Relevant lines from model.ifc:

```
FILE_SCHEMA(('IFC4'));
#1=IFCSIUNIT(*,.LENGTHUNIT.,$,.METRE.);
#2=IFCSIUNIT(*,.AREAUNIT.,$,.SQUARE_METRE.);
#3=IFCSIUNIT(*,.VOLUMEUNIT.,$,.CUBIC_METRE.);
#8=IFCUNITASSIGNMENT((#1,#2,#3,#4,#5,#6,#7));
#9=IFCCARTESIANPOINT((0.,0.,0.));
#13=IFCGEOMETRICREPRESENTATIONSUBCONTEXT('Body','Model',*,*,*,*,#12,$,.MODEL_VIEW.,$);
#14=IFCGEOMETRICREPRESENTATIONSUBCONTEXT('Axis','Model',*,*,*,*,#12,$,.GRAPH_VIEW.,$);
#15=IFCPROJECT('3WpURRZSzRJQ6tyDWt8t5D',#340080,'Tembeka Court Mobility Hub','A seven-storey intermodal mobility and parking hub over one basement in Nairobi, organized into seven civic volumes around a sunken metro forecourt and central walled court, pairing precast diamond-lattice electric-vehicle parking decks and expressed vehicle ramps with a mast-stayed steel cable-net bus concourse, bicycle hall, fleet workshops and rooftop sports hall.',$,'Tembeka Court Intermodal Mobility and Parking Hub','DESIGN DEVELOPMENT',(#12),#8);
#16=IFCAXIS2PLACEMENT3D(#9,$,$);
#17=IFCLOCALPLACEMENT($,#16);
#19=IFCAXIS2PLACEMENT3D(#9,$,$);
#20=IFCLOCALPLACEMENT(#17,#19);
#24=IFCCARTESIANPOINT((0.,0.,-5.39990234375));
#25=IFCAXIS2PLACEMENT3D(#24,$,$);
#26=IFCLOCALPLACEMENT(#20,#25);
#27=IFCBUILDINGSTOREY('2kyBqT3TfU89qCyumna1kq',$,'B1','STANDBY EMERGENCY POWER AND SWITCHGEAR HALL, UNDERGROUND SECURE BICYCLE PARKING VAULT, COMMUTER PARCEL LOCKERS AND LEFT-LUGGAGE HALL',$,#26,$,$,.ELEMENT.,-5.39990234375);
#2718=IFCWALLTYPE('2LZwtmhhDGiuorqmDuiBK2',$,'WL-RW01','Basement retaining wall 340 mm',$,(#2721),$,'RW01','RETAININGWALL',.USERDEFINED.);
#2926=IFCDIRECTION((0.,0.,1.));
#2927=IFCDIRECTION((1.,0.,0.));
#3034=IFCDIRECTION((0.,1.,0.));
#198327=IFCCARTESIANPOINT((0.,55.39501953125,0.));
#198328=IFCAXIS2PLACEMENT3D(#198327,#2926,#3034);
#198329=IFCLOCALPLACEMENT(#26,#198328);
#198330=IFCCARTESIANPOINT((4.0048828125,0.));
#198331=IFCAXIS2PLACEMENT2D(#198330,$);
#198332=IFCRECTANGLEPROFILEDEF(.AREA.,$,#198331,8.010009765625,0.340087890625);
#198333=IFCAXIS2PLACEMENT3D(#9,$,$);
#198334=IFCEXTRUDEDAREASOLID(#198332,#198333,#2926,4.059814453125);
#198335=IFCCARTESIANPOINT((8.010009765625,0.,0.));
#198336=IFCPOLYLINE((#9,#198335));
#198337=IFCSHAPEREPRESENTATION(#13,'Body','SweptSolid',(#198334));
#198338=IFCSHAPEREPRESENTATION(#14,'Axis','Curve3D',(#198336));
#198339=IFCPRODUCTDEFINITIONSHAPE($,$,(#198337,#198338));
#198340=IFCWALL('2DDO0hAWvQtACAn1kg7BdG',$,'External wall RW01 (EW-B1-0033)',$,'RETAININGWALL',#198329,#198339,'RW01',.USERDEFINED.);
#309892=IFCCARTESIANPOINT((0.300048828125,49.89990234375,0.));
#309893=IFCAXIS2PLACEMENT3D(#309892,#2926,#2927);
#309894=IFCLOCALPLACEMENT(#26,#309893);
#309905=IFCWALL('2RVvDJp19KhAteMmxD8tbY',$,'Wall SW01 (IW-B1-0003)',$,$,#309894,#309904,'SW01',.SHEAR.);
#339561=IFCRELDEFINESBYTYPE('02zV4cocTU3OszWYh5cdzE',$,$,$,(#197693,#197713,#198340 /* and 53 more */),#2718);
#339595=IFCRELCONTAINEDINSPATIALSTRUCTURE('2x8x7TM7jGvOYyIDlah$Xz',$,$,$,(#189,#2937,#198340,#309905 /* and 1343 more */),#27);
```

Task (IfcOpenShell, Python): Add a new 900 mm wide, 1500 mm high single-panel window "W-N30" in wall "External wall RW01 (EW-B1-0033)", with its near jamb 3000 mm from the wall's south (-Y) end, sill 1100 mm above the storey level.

```python
import numpy as np
import ifcopenshell
import ifcopenshell.api.feature
import ifcopenshell.api.geometry
import ifcopenshell.api.root
import ifcopenshell.api.spatial
import ifcopenshell.geom
import ifcopenshell.util.element
import ifcopenshell.util.placement
import ifcopenshell.util.representation
import ifcopenshell.util.shape
import ifcopenshell.util.unit

model = ifcopenshell.open("model.ifc")
unit_scale = ifcopenshell.util.unit.calculate_unit_scale(model)
settings = ifcopenshell.geom.settings()


def volume(element):
    """Net volume in cubic metres, openings subtracted."""
    shape = ifcopenshell.geom.create_shape(settings, element)
    return ifcopenshell.util.shape.get_volume(shape.geometry)


wall = model.by_id(198340)
storey = ifcopenshell.util.element.get_container(wall, ifc_class="IfcBuildingStorey")
context = ifcopenshell.util.representation.get_context(model, "Model", "Body", "MODEL_VIEW")
before = volume(wall)

width, height, from_end, sill = 0.9, 1.5, 3, 1.1  # metres

# The wall runs along its own X axis, and the end named is its -X end.
wall_shape = ifcopenshell.geom.create_shape(settings, wall)
x, y, z = ifcopenshell.util.shape.get_vertices(wall_shape.geometry).T
start = x.min() + from_end
face, thickness = float(y.min()), float(y.max() - y.min())
wall_matrix = ifcopenshell.util.placement.get_local_placement(wall.ObjectPlacement)
level = ifcopenshell.util.placement.get_local_placement(storey.ObjectPlacement)[2, 3]


def in_wall(x, y):
    """Placement at x, y metres in the wall's axes, at sill height."""
    matrix = wall_matrix.copy()
    matrix[:, 3] = wall_matrix @ np.array([x / unit_scale, y / unit_scale, 0.0, 1.0])
    matrix[2, 3] = level + sill / unit_scale
    return matrix


# Opening: a box that overshoots both wall faces by 50 mm.
opening = ifcopenshell.api.root.create_entity(model, ifc_class="IfcOpeningElement", predefined_type="OPENING")
box = ifcopenshell.api.geometry.add_wall_representation(
    model, context=context, length=width, height=height, thickness=thickness + 0.1
)
ifcopenshell.api.geometry.assign_representation(model, product=opening, representation=box)
ifcopenshell.api.geometry.edit_object_placement(model, product=opening, matrix=in_wall(start, face - 0.05), is_si=False)
ifcopenshell.api.feature.add_feature(model, feature=opening, element=wall)

window = ifcopenshell.api.root.create_entity(model, ifc_class="IfcWindow", name="W-N30", predefined_type="WINDOW")
window.OverallWidth, window.OverallHeight = width / unit_scale, height / unit_scale
window.PartitioningType = "SINGLE_PANEL"
body = ifcopenshell.api.geometry.add_window_representation(
    model,
    context=context,
    overall_width=window.OverallWidth,
    overall_height=window.OverallHeight,
    partition_type="SINGLE_PANEL",
)
ifcopenshell.api.geometry.assign_representation(model, product=window, representation=body)
ifcopenshell.api.spatial.assign_container(model, products=[window], relating_structure=storey)
ifcopenshell.api.feature.add_filling(model, opening=opening, element=window)

# Centre the window in the wall's thickness.
ifcopenshell.api.geometry.edit_object_placement(model, product=window, matrix=in_wall(start, face), is_si=False)
window_shape = ifcopenshell.geom.create_shape(settings, window)
depth = ifcopenshell.util.shape.get_vertices(window_shape.geometry)[:, 1]
offset = face + thickness / 2 - (depth.min() + depth.max()) / 2
ifcopenshell.api.geometry.edit_object_placement(model, product=window, matrix=in_wall(start, offset), is_si=False)

after = volume(wall)

print(f"wall volume {before:.3f} -> {after:.3f} m3")

model.write("model-out.ifc")
```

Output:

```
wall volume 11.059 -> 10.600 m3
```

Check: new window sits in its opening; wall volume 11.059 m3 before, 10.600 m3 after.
